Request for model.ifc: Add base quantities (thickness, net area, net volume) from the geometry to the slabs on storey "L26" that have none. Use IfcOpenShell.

First a look at what the model holds.

```python
import ifcopenshell
import ifcopenshell.util.element
import ifcopenshell.util.unit

model = ifcopenshell.open("model.ifc")
print(model.schema)
for unit_type in ("LENGTHUNIT", "AREAUNIT", "VOLUMEUNIT"):
    print(unit_type, ifcopenshell.util.unit.calculate_unit_scale(model, unit_type))
storey = next(s for s in model.by_type("IfcBuildingStorey") if s.Name == "L26")
slabs = [e for e in ifcopenshell.util.element.get_decomposition(storey) if e.is_a("IfcSlab")]
for e in sorted(slabs, key=lambda e: e.id()):
    print(e.id(), e.is_a(), e.Name, list(ifcopenshell.util.element.get_psets(e, qtos_only=True)), sep=" | ")
```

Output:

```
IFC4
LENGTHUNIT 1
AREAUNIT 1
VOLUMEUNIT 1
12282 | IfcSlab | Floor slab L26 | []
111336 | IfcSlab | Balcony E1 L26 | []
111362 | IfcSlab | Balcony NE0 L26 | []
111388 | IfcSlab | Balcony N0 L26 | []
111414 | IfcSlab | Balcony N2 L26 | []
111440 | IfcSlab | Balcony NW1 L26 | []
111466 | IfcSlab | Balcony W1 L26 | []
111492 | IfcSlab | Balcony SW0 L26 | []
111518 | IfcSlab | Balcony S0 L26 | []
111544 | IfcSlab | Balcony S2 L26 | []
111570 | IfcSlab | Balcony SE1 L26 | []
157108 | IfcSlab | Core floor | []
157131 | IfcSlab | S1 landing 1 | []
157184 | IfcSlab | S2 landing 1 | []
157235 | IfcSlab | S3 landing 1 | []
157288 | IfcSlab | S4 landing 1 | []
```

```python
import ifcopenshell
import ifcopenshell.api.pset
import ifcopenshell.geom
import ifcopenshell.util.element
import ifcopenshell.util.shape
import ifcopenshell.util.unit

model = ifcopenshell.open("model.ifc")
unit_scale = ifcopenshell.util.unit.calculate_unit_scale(model)
area_scale = ifcopenshell.util.unit.calculate_unit_scale(model, "AREAUNIT")
volume_scale = ifcopenshell.util.unit.calculate_unit_scale(model, "VOLUMEUNIT")
settings = ifcopenshell.geom.settings()

storey = next(s for s in model.by_type("IfcBuildingStorey") if s.Name == "L26")
slabs = [e for e in ifcopenshell.util.element.get_decomposition(storey) if e.is_a("IfcSlab")]

for e in sorted(slabs, key=lambda e: e.id()):
    if ifcopenshell.util.element.get_psets(e, qtos_only=True, should_inherit=False):
        continue
    # Geometry comes back in metres, in the element's own axes.
    shape = ifcopenshell.geom.create_shape(settings, e)
    values = {
        "Width": ifcopenshell.util.shape.get_z(shape.geometry) / unit_scale,
        "NetArea": ifcopenshell.util.shape.get_footprint_area(shape.geometry) / area_scale,
        "NetVolume": ifcopenshell.util.shape.get_volume(shape.geometry) / volume_scale,
    }
    qto = ifcopenshell.api.pset.add_qto(model, product=e, name="Qto_SlabBaseQuantities")
    ifcopenshell.api.pset.edit_qto(model, qto=qto, properties=values)
    print(e.id(), {k: round(v, 3) for k, v in values.items()})

model.write("model-out.ifc")
```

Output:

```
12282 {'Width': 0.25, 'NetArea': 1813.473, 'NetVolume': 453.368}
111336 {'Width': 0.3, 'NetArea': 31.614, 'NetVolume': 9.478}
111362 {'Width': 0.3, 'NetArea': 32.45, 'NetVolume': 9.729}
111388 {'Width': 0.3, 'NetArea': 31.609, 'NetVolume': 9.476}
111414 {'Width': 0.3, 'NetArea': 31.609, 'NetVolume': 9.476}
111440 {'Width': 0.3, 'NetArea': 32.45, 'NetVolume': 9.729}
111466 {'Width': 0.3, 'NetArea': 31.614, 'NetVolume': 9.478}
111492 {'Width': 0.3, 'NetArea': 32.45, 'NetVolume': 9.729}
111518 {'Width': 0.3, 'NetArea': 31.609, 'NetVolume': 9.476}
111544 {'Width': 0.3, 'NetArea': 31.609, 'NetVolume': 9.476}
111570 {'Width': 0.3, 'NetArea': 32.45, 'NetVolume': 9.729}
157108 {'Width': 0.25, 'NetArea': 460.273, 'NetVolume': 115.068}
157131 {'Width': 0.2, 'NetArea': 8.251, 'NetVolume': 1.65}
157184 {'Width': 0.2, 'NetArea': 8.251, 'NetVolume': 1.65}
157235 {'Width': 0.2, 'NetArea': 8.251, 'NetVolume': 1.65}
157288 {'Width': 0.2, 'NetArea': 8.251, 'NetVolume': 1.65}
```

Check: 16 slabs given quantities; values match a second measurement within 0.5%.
